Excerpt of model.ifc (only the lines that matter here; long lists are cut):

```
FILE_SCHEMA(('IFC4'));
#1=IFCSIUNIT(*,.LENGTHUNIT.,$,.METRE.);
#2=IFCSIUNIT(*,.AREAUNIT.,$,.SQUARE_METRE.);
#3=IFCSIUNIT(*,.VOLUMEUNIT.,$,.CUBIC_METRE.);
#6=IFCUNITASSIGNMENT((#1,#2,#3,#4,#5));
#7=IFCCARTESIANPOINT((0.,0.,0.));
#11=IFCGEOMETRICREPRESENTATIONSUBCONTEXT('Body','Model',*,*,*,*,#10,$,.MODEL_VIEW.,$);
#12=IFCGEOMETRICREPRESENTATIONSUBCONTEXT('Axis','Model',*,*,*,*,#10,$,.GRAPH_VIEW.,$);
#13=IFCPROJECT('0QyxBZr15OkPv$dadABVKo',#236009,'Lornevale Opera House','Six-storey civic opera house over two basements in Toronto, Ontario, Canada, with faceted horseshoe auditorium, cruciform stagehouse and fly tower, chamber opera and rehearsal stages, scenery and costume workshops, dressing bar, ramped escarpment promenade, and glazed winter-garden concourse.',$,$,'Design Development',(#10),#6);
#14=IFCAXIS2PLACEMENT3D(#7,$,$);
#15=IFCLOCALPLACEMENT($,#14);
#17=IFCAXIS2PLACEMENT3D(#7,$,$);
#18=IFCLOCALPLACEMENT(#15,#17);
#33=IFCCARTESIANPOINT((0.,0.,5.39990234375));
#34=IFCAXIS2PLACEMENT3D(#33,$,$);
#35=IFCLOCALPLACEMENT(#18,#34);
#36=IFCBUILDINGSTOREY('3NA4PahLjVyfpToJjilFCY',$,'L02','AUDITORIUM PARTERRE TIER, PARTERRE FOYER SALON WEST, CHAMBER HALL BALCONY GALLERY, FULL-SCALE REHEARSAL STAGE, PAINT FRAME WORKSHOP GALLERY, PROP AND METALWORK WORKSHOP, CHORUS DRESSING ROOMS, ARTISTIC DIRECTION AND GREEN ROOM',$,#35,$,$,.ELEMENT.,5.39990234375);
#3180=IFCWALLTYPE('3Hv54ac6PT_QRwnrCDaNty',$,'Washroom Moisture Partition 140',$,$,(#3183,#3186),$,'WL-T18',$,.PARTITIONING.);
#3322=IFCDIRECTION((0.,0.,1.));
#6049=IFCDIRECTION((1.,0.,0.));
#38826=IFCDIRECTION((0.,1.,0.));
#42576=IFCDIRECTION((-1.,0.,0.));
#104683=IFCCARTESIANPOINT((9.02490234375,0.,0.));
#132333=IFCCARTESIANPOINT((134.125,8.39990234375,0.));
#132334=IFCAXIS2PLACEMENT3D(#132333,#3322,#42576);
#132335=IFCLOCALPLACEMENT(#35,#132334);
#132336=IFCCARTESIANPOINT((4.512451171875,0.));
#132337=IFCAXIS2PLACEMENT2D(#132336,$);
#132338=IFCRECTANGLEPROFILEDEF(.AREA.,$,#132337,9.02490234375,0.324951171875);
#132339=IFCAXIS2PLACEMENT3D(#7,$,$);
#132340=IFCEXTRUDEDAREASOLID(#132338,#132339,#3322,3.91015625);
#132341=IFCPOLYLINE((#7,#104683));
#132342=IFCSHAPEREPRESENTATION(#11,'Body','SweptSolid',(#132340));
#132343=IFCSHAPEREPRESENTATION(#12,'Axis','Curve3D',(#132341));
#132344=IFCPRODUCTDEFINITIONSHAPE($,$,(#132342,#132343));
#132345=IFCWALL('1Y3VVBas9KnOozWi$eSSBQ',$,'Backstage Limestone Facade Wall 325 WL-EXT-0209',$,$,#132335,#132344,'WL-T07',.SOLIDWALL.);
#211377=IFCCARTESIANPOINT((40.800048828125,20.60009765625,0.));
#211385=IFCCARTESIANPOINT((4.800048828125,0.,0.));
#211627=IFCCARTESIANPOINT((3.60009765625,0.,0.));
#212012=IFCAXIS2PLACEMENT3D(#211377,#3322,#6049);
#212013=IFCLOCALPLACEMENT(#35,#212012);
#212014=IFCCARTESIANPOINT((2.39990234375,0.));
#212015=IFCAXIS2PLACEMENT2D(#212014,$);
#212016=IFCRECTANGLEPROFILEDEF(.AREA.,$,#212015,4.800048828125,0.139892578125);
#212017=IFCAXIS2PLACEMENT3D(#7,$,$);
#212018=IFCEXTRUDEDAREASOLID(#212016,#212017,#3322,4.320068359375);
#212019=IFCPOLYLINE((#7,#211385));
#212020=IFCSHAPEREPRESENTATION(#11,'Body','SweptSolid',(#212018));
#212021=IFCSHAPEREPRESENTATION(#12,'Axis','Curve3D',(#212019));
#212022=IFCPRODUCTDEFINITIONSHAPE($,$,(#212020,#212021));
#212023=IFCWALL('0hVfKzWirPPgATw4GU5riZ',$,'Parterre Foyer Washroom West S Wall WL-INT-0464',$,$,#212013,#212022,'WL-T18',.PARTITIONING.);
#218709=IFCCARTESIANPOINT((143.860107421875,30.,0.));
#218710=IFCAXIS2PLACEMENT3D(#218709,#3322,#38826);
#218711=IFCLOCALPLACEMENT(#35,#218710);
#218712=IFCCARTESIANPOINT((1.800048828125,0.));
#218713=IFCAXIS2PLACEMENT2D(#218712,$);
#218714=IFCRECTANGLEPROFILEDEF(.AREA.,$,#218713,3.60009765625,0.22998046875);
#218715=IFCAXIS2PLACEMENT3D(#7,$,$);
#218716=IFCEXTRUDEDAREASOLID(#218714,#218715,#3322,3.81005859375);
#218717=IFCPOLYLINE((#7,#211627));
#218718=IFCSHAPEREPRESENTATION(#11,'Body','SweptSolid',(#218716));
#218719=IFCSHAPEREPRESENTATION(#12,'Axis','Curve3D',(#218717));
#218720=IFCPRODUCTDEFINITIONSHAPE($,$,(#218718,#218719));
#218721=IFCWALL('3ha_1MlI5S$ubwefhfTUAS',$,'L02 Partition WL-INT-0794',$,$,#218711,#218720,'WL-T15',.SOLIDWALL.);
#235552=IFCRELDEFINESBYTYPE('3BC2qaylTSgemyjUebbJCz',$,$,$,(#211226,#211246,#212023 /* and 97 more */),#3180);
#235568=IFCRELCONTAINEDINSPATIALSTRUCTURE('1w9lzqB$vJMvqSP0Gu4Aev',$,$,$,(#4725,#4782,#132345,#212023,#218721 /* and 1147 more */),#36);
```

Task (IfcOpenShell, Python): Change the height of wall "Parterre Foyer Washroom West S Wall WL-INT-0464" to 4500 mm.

```python
import ifcopenshell
import ifcopenshell.geom
import ifcopenshell.util.representation
import ifcopenshell.util.shape
import ifcopenshell.util.unit

model = ifcopenshell.open("model.ifc")
unit_scale = ifcopenshell.util.unit.calculate_unit_scale(model)
settings = ifcopenshell.geom.settings()


def volume(element):
    """Net volume in cubic metres, openings subtracted."""
    shape = ifcopenshell.geom.create_shape(settings, element)
    return ifcopenshell.util.shape.get_volume(shape.geometry)


wall = model.by_guid("0hVfKzWirPPgATw4GU5riZ")
before = volume(wall)

body = ifcopenshell.util.representation.get_representation(wall, "Model", "Body")
solid = body.Items[0]
old_height = solid.Depth
solid.Depth = 4.5 / unit_scale
after = volume(wall)

print(f"height {old_height:g} -> {solid.Depth:g}, volume {before:.3f} -> {after:.3f} m3")

model.write("model_v2.ifc")
```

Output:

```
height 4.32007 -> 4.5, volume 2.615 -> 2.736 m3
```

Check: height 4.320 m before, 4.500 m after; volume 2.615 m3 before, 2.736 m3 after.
